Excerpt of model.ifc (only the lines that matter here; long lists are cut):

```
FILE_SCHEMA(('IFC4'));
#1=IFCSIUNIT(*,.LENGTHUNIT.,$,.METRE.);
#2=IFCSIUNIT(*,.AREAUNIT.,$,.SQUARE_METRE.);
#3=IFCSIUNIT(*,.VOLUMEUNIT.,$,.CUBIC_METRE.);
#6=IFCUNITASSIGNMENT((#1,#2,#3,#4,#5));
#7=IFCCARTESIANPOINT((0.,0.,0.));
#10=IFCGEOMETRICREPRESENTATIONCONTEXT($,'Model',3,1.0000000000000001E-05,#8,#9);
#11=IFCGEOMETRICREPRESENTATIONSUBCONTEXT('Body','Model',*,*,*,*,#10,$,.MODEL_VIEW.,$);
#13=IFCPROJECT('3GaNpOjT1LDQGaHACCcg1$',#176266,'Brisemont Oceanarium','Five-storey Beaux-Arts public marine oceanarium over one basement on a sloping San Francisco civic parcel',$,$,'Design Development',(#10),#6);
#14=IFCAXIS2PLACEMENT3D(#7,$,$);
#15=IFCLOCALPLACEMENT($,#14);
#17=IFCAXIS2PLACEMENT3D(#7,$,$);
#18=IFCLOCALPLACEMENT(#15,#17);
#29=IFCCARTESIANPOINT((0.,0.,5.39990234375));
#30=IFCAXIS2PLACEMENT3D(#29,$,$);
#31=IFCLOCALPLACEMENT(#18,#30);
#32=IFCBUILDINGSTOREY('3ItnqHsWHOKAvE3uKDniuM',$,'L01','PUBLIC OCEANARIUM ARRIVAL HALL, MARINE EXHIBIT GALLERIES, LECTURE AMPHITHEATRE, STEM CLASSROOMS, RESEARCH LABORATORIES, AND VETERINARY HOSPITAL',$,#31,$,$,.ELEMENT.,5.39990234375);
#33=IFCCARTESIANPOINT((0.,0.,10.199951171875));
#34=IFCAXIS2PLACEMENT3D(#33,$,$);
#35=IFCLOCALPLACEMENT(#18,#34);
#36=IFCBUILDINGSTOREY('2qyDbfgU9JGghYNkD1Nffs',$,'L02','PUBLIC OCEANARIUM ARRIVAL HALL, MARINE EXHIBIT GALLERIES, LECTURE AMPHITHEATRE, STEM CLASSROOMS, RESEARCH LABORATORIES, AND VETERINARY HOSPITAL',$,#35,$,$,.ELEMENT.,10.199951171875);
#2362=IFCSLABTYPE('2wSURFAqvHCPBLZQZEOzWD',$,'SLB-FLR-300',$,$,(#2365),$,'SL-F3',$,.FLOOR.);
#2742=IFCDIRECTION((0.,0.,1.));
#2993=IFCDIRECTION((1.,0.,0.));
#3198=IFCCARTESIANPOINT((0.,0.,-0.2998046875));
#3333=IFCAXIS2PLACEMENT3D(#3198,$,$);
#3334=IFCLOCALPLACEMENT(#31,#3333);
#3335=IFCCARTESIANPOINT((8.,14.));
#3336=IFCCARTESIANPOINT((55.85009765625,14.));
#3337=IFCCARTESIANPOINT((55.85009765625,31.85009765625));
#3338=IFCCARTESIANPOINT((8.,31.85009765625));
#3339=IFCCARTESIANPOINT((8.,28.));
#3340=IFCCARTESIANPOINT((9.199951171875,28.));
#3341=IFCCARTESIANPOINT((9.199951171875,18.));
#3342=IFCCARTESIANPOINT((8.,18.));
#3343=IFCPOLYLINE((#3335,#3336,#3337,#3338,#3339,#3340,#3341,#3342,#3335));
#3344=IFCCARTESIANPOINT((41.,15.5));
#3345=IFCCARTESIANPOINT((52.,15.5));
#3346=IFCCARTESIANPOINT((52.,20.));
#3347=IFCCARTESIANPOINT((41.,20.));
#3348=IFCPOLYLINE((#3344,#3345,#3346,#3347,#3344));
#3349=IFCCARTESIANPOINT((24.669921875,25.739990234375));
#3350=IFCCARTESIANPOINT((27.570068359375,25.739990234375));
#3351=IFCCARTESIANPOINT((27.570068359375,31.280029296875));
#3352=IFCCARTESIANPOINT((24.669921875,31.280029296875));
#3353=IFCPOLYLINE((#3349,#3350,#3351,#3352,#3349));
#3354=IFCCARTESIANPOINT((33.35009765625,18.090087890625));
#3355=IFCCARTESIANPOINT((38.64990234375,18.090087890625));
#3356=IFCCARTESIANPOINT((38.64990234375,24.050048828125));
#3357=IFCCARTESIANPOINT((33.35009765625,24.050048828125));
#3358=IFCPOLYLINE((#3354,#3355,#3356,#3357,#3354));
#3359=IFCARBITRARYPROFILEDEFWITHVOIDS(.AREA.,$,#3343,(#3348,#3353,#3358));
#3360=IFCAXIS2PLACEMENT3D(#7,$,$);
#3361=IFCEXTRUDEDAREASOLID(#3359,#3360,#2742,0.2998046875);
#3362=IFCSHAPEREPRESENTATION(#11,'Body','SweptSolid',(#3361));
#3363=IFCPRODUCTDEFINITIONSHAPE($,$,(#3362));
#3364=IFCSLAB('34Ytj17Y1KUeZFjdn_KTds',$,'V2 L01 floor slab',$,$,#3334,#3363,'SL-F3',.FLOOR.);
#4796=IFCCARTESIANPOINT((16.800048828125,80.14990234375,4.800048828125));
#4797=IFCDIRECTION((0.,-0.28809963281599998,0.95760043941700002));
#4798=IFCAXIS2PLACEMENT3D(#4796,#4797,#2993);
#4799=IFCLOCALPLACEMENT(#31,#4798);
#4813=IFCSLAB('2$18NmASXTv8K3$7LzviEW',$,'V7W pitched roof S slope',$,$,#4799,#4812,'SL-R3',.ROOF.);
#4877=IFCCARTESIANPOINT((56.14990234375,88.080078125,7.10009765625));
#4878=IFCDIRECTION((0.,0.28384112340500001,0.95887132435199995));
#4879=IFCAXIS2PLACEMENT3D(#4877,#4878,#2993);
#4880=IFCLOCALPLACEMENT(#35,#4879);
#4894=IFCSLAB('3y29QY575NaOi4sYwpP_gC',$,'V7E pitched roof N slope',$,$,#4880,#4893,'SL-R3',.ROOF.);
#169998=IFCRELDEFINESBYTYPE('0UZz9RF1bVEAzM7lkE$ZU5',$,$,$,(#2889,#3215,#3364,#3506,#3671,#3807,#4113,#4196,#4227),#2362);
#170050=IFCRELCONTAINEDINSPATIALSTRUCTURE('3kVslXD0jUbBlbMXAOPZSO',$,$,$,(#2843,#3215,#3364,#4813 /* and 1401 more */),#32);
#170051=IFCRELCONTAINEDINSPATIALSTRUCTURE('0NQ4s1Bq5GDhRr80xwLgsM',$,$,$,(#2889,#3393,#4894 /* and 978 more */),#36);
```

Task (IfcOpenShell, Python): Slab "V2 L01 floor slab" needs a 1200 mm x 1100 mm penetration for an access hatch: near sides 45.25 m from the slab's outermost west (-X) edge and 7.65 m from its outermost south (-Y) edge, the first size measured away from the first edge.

```python
import numpy as np
import ifcopenshell
import ifcopenshell.api.feature
import ifcopenshell.api.geometry
import ifcopenshell.api.root
import ifcopenshell.geom
import ifcopenshell.util.placement
import ifcopenshell.util.representation
import ifcopenshell.util.shape
import ifcopenshell.util.unit

model = ifcopenshell.open("model.ifc")
unit_scale = ifcopenshell.util.unit.calculate_unit_scale(model)
settings = ifcopenshell.geom.settings()


def volume(element):
    """Net volume in cubic metres, openings subtracted."""
    shape = ifcopenshell.geom.create_shape(settings, element)
    return ifcopenshell.util.shape.get_volume(shape.geometry)


slab = model.by_id(3364)
before = volume(slab)

# Extent in the slab's own axes, in metres. The edges named are its -X and -Y sides.
slab_shape = ifcopenshell.geom.create_shape(settings, slab)
vertices = ifcopenshell.util.shape.get_vertices(slab_shape.geometry)
x_min, y_min, bottom = vertices.min(axis=0)
top = vertices[:, 2].max()

opening = ifcopenshell.api.root.create_entity(model, ifc_class="IfcOpeningElement", name="Access hatch opening", predefined_type="OPENING")
context = ifcopenshell.util.representation.get_context(model, "Model", "Body", "MODEL_VIEW")
width, depth = 1.2, 1.1
outline = [(0.0, 0.0), (width, 0.0), (width, depth), (0.0, depth), (0.0, 0.0)]
# Overshoot both faces by 50 mm so the cut is clean.
shape = ifcopenshell.api.geometry.add_slab_representation(
    model, context=context, depth=top - bottom + 0.1, polyline=outline
)
ifcopenshell.api.geometry.assign_representation(model, product=opening, representation=shape)

matrix = ifcopenshell.util.placement.get_local_placement(slab.ObjectPlacement)
matrix[:, 3] = matrix @ np.append(np.array([x_min + 45.25, y_min + 7.65, bottom - 0.05]) / unit_scale, 1.0)
ifcopenshell.api.geometry.edit_object_placement(model, product=opening, matrix=matrix, is_si=False)
ifcopenshell.api.feature.add_feature(model, feature=opening, element=slab)

after = volume(slab)

print(f"slab volume {before:.3f} -> {after:.3f} m3")

model.write("model_updated.ifc")
```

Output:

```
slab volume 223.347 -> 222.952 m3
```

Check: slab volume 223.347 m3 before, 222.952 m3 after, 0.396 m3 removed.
